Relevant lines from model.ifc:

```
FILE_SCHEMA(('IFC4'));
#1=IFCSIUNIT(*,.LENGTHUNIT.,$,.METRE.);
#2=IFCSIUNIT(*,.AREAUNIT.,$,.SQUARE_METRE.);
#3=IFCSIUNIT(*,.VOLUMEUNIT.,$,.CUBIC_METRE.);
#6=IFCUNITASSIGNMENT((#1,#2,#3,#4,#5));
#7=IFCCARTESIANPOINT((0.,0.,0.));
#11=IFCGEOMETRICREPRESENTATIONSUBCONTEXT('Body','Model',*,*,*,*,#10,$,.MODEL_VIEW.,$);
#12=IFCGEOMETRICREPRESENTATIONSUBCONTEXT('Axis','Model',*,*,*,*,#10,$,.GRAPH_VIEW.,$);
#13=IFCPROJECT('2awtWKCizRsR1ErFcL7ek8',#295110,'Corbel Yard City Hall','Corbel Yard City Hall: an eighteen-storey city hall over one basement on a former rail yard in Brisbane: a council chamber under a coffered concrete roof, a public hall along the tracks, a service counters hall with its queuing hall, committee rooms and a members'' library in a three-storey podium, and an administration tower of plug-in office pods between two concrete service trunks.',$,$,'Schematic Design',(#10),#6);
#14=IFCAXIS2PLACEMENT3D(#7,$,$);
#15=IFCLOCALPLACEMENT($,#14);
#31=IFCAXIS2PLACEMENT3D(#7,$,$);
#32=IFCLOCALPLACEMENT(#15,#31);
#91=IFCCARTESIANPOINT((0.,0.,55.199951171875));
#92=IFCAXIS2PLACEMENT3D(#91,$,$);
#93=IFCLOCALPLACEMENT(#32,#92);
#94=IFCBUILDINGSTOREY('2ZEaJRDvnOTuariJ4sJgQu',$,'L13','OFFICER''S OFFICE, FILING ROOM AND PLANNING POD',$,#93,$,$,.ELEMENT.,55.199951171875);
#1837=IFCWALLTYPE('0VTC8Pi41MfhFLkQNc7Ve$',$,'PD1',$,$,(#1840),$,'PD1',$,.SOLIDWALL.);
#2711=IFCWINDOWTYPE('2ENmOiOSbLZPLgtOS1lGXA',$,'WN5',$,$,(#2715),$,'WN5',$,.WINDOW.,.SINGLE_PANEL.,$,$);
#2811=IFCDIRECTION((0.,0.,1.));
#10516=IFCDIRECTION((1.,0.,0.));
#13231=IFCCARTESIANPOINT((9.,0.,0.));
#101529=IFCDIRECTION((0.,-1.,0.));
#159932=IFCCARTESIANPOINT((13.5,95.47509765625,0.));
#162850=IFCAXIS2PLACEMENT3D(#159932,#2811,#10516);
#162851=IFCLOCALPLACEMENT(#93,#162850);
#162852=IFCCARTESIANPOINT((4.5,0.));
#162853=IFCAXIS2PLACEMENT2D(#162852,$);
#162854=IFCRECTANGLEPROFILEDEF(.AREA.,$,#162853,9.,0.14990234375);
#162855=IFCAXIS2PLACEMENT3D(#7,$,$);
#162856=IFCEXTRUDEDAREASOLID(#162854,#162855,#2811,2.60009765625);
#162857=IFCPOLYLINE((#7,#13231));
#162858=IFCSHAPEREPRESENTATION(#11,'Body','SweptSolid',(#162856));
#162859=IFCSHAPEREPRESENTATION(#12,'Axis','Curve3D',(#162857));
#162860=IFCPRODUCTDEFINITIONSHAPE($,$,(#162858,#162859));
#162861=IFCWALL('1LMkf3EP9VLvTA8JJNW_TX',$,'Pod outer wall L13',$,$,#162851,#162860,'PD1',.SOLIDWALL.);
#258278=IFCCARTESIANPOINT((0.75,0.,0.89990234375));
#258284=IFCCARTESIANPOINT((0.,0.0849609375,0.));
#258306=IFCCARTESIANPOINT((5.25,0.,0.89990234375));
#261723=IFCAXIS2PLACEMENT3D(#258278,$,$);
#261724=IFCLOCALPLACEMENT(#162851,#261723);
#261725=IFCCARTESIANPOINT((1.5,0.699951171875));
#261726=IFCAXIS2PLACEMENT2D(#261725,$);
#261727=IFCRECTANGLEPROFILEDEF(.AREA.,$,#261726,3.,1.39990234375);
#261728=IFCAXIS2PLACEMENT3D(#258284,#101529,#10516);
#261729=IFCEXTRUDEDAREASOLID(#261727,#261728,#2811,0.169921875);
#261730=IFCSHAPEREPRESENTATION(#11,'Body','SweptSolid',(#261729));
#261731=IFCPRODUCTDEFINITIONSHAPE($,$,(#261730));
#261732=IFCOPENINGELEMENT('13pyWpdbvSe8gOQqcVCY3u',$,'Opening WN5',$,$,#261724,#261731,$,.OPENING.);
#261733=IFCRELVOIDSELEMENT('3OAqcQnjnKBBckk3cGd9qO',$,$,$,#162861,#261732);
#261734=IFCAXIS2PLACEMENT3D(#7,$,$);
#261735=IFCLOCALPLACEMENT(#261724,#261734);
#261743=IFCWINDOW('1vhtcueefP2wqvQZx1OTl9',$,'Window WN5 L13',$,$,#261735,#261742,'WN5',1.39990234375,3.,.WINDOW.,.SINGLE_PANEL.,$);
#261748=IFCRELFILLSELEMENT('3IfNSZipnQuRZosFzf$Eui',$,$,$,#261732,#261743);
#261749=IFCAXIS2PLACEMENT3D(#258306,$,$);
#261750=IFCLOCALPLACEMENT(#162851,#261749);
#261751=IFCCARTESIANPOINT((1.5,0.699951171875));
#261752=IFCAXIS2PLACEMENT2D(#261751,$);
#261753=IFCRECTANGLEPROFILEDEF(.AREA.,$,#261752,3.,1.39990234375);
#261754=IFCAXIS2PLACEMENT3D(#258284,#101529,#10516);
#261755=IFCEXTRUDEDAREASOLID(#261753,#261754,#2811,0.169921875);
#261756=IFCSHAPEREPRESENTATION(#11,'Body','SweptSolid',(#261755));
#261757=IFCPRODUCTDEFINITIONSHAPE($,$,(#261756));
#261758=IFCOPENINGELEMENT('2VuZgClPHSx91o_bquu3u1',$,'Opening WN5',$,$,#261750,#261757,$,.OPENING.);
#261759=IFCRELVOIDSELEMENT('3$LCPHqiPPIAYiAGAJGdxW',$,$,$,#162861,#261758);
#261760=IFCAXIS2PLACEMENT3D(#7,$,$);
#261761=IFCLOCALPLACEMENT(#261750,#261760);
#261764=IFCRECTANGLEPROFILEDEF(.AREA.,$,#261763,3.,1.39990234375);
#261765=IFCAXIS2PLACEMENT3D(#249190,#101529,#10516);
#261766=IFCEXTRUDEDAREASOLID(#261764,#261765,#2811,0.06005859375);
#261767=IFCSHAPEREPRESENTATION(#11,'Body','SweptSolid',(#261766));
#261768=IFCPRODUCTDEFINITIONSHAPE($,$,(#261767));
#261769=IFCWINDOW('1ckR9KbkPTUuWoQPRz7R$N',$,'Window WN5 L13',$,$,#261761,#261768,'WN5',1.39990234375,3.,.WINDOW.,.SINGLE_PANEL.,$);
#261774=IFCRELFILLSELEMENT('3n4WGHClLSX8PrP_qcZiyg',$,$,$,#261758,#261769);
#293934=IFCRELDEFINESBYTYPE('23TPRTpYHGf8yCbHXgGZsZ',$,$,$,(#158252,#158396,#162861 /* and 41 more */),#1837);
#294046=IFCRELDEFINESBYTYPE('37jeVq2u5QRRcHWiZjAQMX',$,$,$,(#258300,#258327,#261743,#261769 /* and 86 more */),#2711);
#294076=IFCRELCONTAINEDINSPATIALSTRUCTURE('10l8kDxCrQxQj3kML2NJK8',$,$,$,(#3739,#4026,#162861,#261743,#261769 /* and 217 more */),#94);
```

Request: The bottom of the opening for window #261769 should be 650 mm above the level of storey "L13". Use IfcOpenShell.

```python
import numpy as np
import ifcopenshell
import ifcopenshell.api.geometry
import ifcopenshell.geom
import ifcopenshell.util.element
import ifcopenshell.util.placement
import ifcopenshell.util.shape
import ifcopenshell.util.unit

model = ifcopenshell.open("model.ifc")
unit_scale = ifcopenshell.util.unit.calculate_unit_scale(model)

window = model.by_guid("1ckR9KbkPTUuWoQPRz7R$N")
opening = window.FillsVoids[0].RelatingOpeningElement
storey = ifcopenshell.util.element.get_container(window, ifc_class="IfcBuildingStorey")
level = ifcopenshell.util.placement.get_local_placement(storey.ObjectPlacement)[2, 3]

# The opening's origin need not be at the sill, so measure its lowest point.
shape = ifcopenshell.geom.create_shape(ifcopenshell.geom.settings(), opening)
bottom = ifcopenshell.util.shape.get_shape_bottom_elevation(shape, shape.geometry) / unit_scale
dz = level + 0.65 / unit_scale - bottom

shift = np.array([0.0, 0.0, dz])
# The window is placed relative to its opening, so it follows when the opening moves.
matrix = ifcopenshell.util.placement.get_local_placement(opening.ObjectPlacement)
matrix[:3, 3] += shift
ifcopenshell.api.geometry.edit_object_placement(
    model, product=opening, matrix=matrix, is_si=False, should_transform_children=True
)

print(f"moved by {dz * unit_scale:+.3f} m")

model.write("model_updated.ifc")
```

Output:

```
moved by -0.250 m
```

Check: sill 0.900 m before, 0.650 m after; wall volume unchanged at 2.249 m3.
